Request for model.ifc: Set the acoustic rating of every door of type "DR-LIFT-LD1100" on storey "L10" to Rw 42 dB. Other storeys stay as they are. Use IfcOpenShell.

First a look at what the model holds.

```python
import ifcopenshell
import ifcopenshell.util.element

model = ifcopenshell.open("model.ifc")
print(model.schema)
storey = next(s for s in model.by_type("IfcBuildingStorey") if s.Name == "L10")
doors = [e for e in ifcopenshell.util.element.get_decomposition(storey) if e.is_a("IfcDoor")]
seen = {}
for e in doors:
    element_type = ifcopenshell.util.element.get_type(e)
    key = (element_type.Name if element_type != e and element_type else None, ifcopenshell.util.element.get_pset(e, "Pset_DoorCommon", "AcousticRating"))
    seen[key] = seen.get(key, 0) + 1
for (name, value), count in sorted(seen.items(), key=str):
    print(count, "x", name, "|", value)
```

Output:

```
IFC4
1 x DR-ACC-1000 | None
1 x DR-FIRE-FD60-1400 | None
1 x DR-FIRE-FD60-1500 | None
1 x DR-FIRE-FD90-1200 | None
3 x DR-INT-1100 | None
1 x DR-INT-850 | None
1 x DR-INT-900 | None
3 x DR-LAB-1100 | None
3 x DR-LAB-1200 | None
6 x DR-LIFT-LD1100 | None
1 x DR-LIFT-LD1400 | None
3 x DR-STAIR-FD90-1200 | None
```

```python
import ifcopenshell
import ifcopenshell.api.pset
import ifcopenshell.util.element

model = ifcopenshell.open("model.ifc")

storey = next(s for s in model.by_type("IfcBuildingStorey") if s.Name == "L10")
doors = [e for e in ifcopenshell.util.element.get_decomposition(storey) if e.is_a("IfcDoor")]

count = 0
for e in doors:
    element_type = ifcopenshell.util.element.get_type(e)
    if element_type in (None, e) or element_type.Name != "DR-LIFT-LD1100":
        continue
    # add_pset returns the element's existing set when there is one.
    pset = ifcopenshell.api.pset.add_pset(model, product=e, name="Pset_DoorCommon")
    ifcopenshell.api.pset.edit_pset(model, pset=pset, properties={"AcousticRating": "Rw 42 dB"})
    count += 1

print(count, "doors updated")

model.write("model-out.ifc")
```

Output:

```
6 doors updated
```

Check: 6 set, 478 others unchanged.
